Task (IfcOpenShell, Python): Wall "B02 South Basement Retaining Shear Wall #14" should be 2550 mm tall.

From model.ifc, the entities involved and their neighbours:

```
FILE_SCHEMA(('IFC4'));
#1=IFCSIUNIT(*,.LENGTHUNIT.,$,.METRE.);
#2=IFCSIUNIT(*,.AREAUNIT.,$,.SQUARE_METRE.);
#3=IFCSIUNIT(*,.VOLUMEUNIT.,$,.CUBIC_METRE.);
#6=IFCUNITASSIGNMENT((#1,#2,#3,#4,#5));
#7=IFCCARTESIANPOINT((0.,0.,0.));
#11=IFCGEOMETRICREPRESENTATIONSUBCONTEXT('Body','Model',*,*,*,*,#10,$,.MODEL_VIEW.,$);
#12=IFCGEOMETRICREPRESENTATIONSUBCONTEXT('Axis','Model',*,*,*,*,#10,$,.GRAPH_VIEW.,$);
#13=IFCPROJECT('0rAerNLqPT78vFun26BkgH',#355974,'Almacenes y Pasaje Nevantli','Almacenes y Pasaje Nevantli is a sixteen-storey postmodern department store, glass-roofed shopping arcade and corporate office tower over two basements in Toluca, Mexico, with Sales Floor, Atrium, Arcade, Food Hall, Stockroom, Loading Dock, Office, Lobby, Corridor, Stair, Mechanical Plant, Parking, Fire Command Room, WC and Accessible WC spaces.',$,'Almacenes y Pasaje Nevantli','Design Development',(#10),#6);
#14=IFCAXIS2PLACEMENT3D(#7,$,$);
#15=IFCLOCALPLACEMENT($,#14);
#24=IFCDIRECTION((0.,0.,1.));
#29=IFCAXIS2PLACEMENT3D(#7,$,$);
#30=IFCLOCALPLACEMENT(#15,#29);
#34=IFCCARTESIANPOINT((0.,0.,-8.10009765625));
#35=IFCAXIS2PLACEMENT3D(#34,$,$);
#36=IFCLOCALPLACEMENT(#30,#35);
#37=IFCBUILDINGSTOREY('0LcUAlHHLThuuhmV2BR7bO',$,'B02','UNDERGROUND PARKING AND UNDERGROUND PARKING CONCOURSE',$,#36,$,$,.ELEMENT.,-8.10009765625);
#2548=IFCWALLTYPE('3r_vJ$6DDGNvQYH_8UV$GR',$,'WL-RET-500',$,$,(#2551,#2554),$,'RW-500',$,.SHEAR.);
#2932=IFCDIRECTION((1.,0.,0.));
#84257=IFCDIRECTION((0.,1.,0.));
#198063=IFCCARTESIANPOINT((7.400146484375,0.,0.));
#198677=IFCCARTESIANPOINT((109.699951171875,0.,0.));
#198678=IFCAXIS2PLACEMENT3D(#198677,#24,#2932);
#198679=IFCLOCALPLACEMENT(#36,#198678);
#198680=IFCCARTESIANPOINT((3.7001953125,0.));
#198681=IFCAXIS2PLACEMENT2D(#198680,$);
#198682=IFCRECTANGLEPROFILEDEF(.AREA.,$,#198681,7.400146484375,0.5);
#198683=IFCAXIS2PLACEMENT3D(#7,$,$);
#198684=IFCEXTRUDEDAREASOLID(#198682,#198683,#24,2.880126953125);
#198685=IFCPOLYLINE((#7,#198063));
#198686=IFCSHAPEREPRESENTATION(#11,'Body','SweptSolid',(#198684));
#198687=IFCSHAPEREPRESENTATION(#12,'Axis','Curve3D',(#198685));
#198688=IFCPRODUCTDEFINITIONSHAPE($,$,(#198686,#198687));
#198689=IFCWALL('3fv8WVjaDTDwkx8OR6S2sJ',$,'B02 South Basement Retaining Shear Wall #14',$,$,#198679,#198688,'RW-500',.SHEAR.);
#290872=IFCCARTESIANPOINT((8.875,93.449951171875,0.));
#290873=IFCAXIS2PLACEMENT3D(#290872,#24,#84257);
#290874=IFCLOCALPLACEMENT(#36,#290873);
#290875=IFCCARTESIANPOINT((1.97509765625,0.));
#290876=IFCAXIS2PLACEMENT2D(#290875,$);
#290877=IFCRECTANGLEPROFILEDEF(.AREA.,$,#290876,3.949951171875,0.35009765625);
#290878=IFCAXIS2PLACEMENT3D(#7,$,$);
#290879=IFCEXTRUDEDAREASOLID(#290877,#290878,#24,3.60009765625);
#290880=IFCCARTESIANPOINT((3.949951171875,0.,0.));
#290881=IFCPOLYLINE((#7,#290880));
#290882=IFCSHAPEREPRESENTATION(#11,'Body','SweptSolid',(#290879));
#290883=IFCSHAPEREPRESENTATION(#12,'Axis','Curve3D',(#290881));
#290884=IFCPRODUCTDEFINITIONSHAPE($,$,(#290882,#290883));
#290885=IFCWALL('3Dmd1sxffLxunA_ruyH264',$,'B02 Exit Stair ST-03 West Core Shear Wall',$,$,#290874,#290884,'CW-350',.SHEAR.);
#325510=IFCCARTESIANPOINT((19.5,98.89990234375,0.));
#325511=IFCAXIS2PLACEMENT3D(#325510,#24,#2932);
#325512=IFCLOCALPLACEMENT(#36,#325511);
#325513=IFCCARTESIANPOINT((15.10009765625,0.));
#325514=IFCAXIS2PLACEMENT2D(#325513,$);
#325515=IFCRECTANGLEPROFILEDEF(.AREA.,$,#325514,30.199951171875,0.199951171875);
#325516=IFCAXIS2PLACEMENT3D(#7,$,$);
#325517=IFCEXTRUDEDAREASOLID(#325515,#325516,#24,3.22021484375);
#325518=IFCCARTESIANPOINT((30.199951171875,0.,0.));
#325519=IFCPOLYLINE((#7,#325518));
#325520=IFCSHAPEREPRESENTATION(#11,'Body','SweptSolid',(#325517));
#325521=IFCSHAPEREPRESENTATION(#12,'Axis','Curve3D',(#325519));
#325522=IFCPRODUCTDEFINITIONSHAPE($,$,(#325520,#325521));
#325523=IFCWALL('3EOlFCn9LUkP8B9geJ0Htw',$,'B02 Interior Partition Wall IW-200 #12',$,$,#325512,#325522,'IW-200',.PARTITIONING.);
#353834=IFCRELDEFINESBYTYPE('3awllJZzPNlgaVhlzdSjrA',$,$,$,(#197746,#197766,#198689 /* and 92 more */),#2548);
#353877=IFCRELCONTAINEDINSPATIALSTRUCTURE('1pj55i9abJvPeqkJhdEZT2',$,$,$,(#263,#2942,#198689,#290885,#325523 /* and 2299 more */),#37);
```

```python
import ifcopenshell
import ifcopenshell.geom
import ifcopenshell.util.representation
import ifcopenshell.util.shape
import ifcopenshell.util.unit

model = ifcopenshell.open("model.ifc")
unit_scale = ifcopenshell.util.unit.calculate_unit_scale(model)
settings = ifcopenshell.geom.settings()


def volume(element):
    """Net volume in cubic metres, openings subtracted."""
    shape = ifcopenshell.geom.create_shape(settings, element)
    return ifcopenshell.util.shape.get_volume(shape.geometry)


wall = model.by_id(198689)
before = volume(wall)

body = ifcopenshell.util.representation.get_representation(wall, "Model", "Body")
solid = body.Items[0]
old_height = solid.Depth
solid.Depth = 2.55 / unit_scale
after = volume(wall)

print(f"height {old_height:g} -> {solid.Depth:g}, volume {before:.3f} -> {after:.3f} m3")

model.write("model_edited.ifc")
```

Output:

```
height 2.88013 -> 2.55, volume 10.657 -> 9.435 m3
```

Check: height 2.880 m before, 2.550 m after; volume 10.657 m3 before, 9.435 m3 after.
